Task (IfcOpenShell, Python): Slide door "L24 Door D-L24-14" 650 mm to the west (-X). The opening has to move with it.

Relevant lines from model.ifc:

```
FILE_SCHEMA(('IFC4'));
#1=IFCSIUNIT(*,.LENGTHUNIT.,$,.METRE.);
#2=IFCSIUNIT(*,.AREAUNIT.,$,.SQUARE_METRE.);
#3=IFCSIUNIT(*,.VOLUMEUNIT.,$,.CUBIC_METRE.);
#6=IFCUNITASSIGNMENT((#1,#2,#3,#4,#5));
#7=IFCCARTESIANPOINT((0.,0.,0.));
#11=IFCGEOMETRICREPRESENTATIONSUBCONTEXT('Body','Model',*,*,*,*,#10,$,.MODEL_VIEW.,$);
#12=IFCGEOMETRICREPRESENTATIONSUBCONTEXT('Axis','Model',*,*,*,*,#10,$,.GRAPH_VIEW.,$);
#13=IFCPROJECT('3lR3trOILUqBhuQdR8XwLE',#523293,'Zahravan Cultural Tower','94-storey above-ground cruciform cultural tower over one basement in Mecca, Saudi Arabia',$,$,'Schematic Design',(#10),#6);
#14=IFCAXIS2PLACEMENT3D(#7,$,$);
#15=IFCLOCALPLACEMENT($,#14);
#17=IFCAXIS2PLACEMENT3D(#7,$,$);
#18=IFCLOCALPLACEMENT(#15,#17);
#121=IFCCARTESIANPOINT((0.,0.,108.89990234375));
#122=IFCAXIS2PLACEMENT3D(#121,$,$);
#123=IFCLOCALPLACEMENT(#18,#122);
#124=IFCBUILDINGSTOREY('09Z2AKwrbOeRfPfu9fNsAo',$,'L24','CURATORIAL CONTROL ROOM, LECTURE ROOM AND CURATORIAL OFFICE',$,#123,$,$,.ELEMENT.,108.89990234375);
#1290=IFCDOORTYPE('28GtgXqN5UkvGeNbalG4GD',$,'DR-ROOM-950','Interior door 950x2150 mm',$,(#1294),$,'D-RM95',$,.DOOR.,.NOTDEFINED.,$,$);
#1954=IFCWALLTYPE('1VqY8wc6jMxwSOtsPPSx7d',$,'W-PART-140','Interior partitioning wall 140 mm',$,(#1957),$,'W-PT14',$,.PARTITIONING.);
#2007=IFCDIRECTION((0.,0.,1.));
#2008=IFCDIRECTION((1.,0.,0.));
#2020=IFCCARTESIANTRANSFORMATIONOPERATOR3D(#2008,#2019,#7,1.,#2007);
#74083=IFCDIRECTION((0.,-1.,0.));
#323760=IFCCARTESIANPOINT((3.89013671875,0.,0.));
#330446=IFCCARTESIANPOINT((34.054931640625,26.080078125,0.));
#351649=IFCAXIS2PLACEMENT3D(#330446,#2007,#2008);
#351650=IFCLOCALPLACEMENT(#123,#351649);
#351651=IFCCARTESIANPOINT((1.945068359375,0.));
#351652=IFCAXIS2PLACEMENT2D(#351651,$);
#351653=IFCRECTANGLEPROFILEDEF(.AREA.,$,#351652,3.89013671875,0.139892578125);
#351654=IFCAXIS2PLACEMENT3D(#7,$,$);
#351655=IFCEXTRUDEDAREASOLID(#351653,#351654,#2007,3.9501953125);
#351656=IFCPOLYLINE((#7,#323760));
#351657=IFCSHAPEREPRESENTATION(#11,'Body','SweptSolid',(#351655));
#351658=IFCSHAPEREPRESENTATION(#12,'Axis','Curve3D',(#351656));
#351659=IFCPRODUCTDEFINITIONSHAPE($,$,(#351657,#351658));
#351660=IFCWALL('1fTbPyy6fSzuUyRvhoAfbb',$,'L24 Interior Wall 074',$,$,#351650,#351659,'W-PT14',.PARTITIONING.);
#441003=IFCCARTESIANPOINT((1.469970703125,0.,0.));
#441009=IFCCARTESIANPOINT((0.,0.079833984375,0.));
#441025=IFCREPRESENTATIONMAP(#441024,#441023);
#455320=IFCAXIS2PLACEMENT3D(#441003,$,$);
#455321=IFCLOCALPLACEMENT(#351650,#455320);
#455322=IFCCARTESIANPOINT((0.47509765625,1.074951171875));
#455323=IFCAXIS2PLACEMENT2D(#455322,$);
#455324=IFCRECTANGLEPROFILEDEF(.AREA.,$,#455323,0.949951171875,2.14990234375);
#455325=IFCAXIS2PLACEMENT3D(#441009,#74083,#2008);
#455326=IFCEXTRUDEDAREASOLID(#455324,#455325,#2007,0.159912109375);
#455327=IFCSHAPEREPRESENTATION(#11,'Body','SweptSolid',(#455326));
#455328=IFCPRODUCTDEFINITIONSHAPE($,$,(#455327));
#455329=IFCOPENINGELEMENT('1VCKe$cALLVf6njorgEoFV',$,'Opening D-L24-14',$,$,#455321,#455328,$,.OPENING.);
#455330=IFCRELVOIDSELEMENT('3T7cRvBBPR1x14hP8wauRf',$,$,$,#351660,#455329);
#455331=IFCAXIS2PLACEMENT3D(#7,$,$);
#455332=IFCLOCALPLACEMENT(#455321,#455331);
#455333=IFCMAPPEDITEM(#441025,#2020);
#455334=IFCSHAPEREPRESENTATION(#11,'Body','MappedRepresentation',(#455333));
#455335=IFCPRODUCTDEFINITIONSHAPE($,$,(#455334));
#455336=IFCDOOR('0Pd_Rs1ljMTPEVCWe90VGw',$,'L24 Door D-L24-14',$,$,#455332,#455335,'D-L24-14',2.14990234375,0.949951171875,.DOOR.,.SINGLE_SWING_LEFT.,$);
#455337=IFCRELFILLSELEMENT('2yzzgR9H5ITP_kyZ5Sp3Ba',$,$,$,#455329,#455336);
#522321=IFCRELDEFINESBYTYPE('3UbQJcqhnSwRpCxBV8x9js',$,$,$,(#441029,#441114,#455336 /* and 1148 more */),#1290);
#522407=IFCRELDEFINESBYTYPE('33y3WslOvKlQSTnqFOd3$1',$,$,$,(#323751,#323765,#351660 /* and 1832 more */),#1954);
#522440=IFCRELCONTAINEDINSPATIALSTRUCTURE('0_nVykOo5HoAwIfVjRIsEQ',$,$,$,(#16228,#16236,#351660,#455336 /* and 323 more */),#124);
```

```python
import ifcopenshell
import ifcopenshell.api.geometry
import ifcopenshell.util.placement

model = ifcopenshell.open("model.ifc")

door = model.by_id(455336)
opening = door.FillsVoids[0].RelatingOpeningElement
wall = opening.VoidsElements[0].RelatingBuildingElement

wall_matrix = ifcopenshell.util.placement.get_local_placement(wall.ObjectPlacement)
shift = wall_matrix[:3, 0] * -0.65
before = ifcopenshell.util.placement.get_local_placement(door.ObjectPlacement)[:3, 3].copy()

# The door is placed relative to its opening, so it follows when the opening moves.
matrix = ifcopenshell.util.placement.get_local_placement(opening.ObjectPlacement)
matrix[:3, 3] += shift
ifcopenshell.api.geometry.edit_object_placement(
    model, product=opening, matrix=matrix, is_si=False, should_transform_children=True
)

after = ifcopenshell.util.placement.get_local_placement(door.ObjectPlacement)[:3, 3]
print("door moved by", (after - before).round(3) + 0.0)

model.write("model_updated.ifc")
```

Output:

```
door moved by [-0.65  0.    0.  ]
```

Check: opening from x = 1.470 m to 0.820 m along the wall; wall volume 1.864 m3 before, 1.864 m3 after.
